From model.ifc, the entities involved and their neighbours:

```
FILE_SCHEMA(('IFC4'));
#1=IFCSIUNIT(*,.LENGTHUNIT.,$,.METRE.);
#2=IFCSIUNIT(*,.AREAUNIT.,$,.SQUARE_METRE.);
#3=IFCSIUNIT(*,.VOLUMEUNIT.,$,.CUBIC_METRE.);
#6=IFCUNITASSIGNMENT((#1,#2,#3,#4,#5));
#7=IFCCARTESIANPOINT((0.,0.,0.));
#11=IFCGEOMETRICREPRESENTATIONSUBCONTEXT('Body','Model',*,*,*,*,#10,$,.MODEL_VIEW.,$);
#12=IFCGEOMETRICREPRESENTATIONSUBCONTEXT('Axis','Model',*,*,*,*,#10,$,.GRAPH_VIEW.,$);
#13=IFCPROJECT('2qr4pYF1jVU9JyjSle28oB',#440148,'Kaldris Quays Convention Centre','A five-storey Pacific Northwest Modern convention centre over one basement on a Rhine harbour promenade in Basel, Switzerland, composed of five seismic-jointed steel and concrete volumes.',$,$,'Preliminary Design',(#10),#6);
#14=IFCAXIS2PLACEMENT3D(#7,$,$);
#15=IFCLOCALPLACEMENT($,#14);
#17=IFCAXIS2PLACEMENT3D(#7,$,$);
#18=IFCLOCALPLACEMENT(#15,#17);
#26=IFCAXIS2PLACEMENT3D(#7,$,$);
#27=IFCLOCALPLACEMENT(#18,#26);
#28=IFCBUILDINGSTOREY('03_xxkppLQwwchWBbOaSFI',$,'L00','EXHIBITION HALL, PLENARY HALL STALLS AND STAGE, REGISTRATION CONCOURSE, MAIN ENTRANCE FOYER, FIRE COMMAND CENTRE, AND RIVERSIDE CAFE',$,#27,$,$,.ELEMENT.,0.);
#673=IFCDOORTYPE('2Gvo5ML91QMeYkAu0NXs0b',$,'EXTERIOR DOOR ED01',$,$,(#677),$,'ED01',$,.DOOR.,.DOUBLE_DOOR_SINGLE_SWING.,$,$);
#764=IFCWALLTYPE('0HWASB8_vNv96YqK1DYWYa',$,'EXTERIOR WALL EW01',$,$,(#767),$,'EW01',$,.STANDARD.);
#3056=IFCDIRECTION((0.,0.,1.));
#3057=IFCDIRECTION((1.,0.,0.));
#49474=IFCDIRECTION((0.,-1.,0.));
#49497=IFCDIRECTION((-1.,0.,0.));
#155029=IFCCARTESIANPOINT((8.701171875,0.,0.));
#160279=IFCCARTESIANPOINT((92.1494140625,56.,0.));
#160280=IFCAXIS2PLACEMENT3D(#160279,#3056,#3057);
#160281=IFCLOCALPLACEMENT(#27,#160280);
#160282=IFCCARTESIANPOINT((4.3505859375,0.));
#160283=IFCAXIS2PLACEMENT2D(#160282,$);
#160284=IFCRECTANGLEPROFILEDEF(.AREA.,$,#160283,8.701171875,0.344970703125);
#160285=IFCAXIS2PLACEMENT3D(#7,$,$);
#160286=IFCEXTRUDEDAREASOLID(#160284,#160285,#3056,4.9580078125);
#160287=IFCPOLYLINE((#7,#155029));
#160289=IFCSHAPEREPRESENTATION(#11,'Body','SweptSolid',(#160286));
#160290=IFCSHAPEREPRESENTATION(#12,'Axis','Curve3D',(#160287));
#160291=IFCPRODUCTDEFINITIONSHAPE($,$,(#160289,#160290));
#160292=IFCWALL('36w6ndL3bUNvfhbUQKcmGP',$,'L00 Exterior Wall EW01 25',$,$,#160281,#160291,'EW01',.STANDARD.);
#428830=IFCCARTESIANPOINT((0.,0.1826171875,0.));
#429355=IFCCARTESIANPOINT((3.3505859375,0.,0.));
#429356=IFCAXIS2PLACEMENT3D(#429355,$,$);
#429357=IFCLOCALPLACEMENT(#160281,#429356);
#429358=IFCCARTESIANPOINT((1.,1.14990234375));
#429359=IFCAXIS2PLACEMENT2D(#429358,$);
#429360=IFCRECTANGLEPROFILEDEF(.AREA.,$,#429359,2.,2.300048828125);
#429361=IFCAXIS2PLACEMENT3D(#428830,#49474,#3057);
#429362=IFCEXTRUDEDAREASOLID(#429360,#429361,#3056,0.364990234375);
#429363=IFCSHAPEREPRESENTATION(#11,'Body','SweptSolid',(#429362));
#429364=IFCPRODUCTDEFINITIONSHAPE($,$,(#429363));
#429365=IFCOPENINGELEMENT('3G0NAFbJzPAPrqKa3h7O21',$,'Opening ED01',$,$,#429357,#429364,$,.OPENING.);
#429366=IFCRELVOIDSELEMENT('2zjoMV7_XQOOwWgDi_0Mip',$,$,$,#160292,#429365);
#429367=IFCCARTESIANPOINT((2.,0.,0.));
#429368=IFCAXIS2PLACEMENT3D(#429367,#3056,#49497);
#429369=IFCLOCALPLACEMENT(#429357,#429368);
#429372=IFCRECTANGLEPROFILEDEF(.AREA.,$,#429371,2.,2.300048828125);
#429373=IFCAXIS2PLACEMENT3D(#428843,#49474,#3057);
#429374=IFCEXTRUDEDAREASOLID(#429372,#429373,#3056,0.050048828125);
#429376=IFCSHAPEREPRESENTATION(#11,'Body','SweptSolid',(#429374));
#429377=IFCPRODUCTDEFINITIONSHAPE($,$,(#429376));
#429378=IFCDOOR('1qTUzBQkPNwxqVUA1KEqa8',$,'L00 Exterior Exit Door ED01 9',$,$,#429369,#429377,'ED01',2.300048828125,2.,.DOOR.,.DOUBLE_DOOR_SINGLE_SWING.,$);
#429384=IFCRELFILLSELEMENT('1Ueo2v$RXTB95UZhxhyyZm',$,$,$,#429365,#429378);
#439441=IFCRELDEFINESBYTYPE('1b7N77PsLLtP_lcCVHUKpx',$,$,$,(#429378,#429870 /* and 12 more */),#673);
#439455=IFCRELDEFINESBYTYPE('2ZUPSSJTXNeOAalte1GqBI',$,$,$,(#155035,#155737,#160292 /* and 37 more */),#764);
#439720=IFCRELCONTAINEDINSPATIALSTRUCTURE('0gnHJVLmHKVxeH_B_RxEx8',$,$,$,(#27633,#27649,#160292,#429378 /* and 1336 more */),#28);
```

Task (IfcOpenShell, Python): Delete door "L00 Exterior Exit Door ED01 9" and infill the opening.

```python
import ifcopenshell
import ifcopenshell.api.feature
import ifcopenshell.api.root
import ifcopenshell.geom
import ifcopenshell.util.shape

model = ifcopenshell.open("model.ifc")
settings = ifcopenshell.geom.settings()


def volume(element):
    """Net volume in cubic metres, openings subtracted."""
    shape = ifcopenshell.geom.create_shape(settings, element)
    return ifcopenshell.util.shape.get_volume(shape.geometry)


door = model.by_guid("1qTUzBQkPNwxqVUA1KEqa8")
opening = door.FillsVoids[0].RelatingOpeningElement
wall = opening.VoidsElements[0].RelatingBuildingElement
before = volume(wall)

ifcopenshell.api.root.remove_product(model, product=door)
ifcopenshell.api.feature.remove_feature(model, feature=opening)

after = volume(wall)

print(f"wall volume {before:.3f} -> {after:.3f} m3")

model.write("model_edited.ifc")
```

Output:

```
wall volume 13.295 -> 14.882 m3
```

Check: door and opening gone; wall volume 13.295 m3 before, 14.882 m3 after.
